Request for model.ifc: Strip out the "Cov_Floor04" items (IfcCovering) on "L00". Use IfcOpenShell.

First a look at what the model holds.

```python
import ifcopenshell
import ifcopenshell.util.element

model = ifcopenshell.open("model.ifc")
print(model.schema)
storey = next(s for s in model.by_type("IfcBuildingStorey") if s.Name == "L00")
coverings = [e for e in ifcopenshell.util.element.get_decomposition(storey) if e.is_a("IfcCovering")]
seen = {}
for e in coverings:
    element_type = ifcopenshell.util.element.get_type(e)
    name = element_type.Name if element_type not in (None, e) else None
    seen[name] = seen.get(name, 0) + 1
for name, count in sorted(seen.items(), key=str):
    print(count, "x", name)
```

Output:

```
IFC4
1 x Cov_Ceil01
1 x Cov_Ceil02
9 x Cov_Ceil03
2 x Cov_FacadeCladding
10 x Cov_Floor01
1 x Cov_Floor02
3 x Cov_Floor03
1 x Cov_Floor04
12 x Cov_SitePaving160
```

```python
import ifcopenshell
import ifcopenshell.api.root
import ifcopenshell.util.element

model = ifcopenshell.open("model.ifc")

storey = next(s for s in model.by_type("IfcBuildingStorey") if s.Name == "L00")
coverings = [e for e in ifcopenshell.util.element.get_decomposition(storey) if e.is_a("IfcCovering")]
targets = [e for e in coverings if (t := ifcopenshell.util.element.get_type(e)) not in (None, e) and t.Name == "Cov_Floor04"]

for e in targets:
    ifcopenshell.api.root.remove_product(model, product=e)
print(len(targets), "removed")

model.write("model_v2.ifc")
```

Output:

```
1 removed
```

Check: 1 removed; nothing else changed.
